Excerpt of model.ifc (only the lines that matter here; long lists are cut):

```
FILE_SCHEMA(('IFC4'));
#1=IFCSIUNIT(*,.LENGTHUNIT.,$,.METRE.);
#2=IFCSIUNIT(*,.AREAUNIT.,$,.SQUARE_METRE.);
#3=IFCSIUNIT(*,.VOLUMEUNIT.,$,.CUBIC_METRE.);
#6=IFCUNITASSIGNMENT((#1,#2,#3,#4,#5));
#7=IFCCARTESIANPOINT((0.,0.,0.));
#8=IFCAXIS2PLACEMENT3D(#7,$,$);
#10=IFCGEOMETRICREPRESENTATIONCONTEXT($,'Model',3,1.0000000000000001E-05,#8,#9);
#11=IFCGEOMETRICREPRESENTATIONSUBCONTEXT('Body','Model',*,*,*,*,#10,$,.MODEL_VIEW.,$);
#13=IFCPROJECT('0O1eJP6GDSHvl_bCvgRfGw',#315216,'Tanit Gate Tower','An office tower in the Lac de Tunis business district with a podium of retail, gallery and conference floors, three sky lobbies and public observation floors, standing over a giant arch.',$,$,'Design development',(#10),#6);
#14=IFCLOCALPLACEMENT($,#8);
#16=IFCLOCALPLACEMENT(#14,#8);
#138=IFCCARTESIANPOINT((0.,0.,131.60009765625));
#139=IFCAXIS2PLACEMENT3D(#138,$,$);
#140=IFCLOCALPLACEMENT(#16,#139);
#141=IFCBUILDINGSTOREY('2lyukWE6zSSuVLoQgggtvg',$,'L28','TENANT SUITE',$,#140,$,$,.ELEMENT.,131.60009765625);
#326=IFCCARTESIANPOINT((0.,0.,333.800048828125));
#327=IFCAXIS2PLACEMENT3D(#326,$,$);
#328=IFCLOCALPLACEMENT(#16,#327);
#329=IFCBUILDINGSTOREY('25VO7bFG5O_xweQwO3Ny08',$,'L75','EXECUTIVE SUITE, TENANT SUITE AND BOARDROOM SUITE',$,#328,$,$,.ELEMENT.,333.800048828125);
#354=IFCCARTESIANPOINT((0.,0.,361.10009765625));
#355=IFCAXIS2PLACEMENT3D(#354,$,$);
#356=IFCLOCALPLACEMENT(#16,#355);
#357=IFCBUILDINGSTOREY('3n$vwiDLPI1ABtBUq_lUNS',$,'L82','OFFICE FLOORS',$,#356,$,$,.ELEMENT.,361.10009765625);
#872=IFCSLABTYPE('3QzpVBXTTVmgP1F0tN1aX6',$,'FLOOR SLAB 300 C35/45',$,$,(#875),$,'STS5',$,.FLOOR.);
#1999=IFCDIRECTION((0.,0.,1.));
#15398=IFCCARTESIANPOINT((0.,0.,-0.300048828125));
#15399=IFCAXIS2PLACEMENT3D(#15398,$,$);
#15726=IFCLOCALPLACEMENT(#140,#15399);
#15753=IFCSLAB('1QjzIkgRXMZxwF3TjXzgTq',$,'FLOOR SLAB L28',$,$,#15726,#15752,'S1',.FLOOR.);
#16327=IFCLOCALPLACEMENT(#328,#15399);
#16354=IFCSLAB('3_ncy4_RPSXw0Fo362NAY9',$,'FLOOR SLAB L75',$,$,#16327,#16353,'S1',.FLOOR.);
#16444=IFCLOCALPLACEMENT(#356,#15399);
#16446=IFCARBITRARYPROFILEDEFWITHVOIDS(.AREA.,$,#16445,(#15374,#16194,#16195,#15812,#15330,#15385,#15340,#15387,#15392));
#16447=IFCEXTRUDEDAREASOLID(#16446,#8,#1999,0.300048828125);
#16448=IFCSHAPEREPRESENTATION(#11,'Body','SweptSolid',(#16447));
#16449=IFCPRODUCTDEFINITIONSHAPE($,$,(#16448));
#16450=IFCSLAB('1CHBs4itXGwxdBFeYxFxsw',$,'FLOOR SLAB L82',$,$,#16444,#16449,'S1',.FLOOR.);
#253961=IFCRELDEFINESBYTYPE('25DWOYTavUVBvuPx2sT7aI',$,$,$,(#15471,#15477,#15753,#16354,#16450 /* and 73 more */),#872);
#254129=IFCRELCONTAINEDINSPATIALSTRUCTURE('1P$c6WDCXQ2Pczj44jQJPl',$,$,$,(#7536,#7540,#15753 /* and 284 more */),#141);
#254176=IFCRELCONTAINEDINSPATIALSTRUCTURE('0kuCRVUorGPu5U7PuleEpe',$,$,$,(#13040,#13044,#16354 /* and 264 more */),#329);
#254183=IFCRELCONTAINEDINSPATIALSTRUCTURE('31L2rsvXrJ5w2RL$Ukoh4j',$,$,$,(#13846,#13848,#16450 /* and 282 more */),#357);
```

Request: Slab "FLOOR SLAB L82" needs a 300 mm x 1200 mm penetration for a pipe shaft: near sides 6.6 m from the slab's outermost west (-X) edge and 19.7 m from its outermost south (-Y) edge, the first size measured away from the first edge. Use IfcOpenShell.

```python
import numpy as np
import ifcopenshell
import ifcopenshell.api.feature
import ifcopenshell.api.geometry
import ifcopenshell.api.root
import ifcopenshell.geom
import ifcopenshell.util.placement
import ifcopenshell.util.representation
import ifcopenshell.util.shape
import ifcopenshell.util.unit

model = ifcopenshell.open("model.ifc")
unit_scale = ifcopenshell.util.unit.calculate_unit_scale(model)
settings = ifcopenshell.geom.settings()


def volume(element):
    """Net volume in cubic metres, openings subtracted."""
    shape = ifcopenshell.geom.create_shape(settings, element)
    return ifcopenshell.util.shape.get_volume(shape.geometry)


slab = model.by_id(16450)
before = volume(slab)

# Extent in the slab's own axes, in metres. The edges named are its -X and -Y sides.
slab_shape = ifcopenshell.geom.create_shape(settings, slab)
vertices = ifcopenshell.util.shape.get_vertices(slab_shape.geometry)
x_min, y_min, bottom = vertices.min(axis=0)
top = vertices[:, 2].max()

opening = ifcopenshell.api.root.create_entity(model, ifc_class="IfcOpeningElement", name="Pipe shaft opening", predefined_type="OPENING")
context = ifcopenshell.util.representation.get_context(model, "Model", "Body", "MODEL_VIEW")
width, depth = 0.3, 1.2
outline = [(0.0, 0.0), (width, 0.0), (width, depth), (0.0, depth), (0.0, 0.0)]
# Overshoot both faces by 50 mm so the cut is clean.
shape = ifcopenshell.api.geometry.add_slab_representation(
    model, context=context, depth=top - bottom + 0.1, polyline=outline
)
ifcopenshell.api.geometry.assign_representation(model, product=opening, representation=shape)

matrix = ifcopenshell.util.placement.get_local_placement(slab.ObjectPlacement)
matrix[:, 3] = matrix @ np.append(np.array([x_min + 6.6, y_min + 19.7, bottom - 0.05]) / unit_scale, 1.0)
ifcopenshell.api.geometry.edit_object_placement(model, product=opening, matrix=matrix, is_si=False)
ifcopenshell.api.feature.add_feature(model, feature=opening, element=slab)

after = volume(slab)

print(f"slab volume {before:.3f} -> {after:.3f} m3")

model.write("model_rev.ifc")
```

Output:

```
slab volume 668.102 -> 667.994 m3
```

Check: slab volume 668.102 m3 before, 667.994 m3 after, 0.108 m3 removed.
